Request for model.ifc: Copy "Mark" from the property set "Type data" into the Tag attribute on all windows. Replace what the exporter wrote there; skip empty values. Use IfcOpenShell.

First a look at what the model holds.

```python
import ifcopenshell
import ifcopenshell.util.element

model = ifcopenshell.open("model.ifc")
print(model.schema)
windows = model.by_type("IfcWindow")
print(len(windows), "windows")
for e in windows[:8]:
    source = ifcopenshell.util.element.get_pset(e, "Type data", "Mark")
    target = e.Tag
    print(e.id(), repr(source), repr(target), sep=" | ")
```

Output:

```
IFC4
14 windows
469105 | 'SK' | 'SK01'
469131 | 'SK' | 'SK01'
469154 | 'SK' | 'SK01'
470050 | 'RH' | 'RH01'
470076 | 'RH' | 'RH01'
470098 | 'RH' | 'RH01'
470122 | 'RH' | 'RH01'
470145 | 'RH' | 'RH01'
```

```python
import ifcopenshell
import ifcopenshell.util.element

model = ifcopenshell.open("model.ifc")

count = 0
for e in model.by_type("IfcWindow"):
    value = ifcopenshell.util.element.get_pset(e, "Type data", "Mark")
    current = e.Tag
    if not value or not value.strip() or current == value:
        continue
    e.Tag = value
    count += 1

print(count, "windows updated")

model.write("model-out.ifc")
```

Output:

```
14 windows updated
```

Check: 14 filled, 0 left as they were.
